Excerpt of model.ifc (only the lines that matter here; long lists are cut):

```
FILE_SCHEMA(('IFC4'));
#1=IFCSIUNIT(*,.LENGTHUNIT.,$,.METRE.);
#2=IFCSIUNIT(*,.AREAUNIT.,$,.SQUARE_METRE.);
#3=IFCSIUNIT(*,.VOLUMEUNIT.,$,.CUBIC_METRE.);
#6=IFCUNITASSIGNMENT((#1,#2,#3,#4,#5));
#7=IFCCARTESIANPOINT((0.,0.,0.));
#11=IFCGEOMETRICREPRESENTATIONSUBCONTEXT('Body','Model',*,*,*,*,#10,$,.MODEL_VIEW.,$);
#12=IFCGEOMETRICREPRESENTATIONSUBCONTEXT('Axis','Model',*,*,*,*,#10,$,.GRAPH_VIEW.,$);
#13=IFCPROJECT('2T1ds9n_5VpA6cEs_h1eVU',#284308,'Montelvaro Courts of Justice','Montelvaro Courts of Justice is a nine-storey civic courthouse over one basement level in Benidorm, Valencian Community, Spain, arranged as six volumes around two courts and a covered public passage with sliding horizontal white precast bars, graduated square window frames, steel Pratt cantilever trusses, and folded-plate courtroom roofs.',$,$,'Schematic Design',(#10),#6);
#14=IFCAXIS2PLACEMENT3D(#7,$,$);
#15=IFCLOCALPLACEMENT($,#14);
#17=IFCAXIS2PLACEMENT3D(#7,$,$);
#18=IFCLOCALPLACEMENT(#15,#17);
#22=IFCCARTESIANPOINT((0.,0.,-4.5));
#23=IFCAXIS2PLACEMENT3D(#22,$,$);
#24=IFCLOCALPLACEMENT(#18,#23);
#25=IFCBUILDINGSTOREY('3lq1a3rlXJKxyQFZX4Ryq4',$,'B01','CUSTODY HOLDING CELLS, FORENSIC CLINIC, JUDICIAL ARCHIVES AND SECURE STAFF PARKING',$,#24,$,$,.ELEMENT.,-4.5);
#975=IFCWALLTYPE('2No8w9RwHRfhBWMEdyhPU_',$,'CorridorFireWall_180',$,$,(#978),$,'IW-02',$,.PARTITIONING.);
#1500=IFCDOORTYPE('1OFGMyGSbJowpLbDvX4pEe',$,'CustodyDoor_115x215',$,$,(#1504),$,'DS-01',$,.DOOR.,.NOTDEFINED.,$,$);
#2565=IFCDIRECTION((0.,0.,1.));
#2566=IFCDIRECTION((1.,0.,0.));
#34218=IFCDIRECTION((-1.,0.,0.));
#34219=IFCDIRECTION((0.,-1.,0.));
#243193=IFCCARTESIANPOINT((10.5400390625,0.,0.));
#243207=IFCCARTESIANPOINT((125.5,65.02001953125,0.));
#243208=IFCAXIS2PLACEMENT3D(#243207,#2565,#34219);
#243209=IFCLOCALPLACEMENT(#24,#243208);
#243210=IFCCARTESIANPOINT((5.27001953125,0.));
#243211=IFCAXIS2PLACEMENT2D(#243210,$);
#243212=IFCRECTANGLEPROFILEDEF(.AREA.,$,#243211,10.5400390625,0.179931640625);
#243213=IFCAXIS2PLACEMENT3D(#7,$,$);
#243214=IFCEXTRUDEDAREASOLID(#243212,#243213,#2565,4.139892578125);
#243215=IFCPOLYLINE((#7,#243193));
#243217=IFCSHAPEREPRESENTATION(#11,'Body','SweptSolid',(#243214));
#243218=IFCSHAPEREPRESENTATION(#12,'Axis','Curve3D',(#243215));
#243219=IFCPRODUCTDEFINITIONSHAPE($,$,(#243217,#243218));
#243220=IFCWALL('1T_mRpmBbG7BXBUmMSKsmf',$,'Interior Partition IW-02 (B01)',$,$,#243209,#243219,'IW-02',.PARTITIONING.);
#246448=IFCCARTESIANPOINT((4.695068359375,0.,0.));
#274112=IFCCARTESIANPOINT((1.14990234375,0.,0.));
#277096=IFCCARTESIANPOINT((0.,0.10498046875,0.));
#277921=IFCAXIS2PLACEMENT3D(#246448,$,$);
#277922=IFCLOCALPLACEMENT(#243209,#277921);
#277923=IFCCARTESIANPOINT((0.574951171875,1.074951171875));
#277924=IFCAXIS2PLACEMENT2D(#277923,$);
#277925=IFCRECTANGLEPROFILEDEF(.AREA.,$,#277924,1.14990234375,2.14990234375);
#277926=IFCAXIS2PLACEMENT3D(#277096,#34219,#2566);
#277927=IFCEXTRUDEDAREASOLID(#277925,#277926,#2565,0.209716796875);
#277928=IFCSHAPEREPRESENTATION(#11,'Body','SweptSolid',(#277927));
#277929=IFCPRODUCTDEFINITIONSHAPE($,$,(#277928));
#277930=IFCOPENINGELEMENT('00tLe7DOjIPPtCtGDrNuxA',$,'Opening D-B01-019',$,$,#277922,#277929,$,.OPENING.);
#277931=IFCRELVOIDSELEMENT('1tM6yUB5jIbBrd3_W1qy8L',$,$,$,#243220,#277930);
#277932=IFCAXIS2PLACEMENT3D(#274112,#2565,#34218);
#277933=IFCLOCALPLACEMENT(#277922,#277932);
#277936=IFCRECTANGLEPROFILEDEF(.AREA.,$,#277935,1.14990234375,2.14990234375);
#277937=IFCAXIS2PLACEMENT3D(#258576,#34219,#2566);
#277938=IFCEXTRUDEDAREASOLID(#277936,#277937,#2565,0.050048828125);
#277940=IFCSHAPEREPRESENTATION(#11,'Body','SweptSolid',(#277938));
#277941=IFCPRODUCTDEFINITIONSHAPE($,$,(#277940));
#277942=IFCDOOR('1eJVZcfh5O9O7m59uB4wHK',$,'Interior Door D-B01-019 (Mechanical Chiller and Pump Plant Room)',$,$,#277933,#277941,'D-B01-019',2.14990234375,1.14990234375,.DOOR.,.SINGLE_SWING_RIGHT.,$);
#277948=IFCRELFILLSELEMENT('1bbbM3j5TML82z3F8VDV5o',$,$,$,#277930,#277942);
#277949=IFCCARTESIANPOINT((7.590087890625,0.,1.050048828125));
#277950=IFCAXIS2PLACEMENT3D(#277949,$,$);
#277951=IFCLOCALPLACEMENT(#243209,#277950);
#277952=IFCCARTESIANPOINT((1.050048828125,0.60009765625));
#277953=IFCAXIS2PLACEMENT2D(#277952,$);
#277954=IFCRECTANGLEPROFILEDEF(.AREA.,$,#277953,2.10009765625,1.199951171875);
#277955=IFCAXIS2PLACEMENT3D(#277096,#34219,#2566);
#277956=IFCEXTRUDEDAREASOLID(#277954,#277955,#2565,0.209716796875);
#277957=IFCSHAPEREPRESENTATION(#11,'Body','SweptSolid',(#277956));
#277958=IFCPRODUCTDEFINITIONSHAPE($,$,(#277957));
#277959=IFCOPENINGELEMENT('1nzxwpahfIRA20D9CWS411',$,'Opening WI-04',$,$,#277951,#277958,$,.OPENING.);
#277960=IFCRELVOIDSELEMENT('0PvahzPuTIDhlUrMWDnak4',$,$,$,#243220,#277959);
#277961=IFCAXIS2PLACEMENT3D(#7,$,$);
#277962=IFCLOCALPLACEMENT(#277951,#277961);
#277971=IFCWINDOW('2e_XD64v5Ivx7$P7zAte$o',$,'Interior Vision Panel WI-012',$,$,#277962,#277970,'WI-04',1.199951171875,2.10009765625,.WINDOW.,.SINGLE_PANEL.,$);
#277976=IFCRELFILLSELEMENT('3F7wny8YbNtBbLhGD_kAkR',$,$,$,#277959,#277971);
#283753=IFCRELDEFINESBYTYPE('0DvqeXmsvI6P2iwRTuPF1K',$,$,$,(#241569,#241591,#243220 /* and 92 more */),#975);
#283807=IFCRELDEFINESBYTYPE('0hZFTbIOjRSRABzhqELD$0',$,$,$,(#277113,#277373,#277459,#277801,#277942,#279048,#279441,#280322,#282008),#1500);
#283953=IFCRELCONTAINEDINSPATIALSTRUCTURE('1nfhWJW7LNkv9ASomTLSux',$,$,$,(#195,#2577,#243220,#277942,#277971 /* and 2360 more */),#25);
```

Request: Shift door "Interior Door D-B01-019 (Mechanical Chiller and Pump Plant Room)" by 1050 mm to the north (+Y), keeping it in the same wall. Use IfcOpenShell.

```python
import ifcopenshell
import ifcopenshell.api.geometry
import ifcopenshell.util.placement

model = ifcopenshell.open("model.ifc")

door = model.by_guid("1eJVZcfh5O9O7m59uB4wHK")
opening = door.FillsVoids[0].RelatingOpeningElement
wall = opening.VoidsElements[0].RelatingBuildingElement

wall_matrix = ifcopenshell.util.placement.get_local_placement(wall.ObjectPlacement)
shift = wall_matrix[:3, 0] * -1.05
before = ifcopenshell.util.placement.get_local_placement(door.ObjectPlacement)[:3, 3].copy()

# The door is placed relative to its opening, so it follows when the opening moves.
matrix = ifcopenshell.util.placement.get_local_placement(opening.ObjectPlacement)
matrix[:3, 3] += shift
ifcopenshell.api.geometry.edit_object_placement(
    model, product=opening, matrix=matrix, is_si=False, should_transform_children=True
)

after = ifcopenshell.util.placement.get_local_placement(door.ObjectPlacement)[:3, 3]
print("door moved by", (after - before).round(3) + 0.0)

model.write("model_updated.ifc")
```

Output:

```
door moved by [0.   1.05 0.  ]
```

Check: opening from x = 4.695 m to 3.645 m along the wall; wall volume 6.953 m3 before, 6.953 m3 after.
